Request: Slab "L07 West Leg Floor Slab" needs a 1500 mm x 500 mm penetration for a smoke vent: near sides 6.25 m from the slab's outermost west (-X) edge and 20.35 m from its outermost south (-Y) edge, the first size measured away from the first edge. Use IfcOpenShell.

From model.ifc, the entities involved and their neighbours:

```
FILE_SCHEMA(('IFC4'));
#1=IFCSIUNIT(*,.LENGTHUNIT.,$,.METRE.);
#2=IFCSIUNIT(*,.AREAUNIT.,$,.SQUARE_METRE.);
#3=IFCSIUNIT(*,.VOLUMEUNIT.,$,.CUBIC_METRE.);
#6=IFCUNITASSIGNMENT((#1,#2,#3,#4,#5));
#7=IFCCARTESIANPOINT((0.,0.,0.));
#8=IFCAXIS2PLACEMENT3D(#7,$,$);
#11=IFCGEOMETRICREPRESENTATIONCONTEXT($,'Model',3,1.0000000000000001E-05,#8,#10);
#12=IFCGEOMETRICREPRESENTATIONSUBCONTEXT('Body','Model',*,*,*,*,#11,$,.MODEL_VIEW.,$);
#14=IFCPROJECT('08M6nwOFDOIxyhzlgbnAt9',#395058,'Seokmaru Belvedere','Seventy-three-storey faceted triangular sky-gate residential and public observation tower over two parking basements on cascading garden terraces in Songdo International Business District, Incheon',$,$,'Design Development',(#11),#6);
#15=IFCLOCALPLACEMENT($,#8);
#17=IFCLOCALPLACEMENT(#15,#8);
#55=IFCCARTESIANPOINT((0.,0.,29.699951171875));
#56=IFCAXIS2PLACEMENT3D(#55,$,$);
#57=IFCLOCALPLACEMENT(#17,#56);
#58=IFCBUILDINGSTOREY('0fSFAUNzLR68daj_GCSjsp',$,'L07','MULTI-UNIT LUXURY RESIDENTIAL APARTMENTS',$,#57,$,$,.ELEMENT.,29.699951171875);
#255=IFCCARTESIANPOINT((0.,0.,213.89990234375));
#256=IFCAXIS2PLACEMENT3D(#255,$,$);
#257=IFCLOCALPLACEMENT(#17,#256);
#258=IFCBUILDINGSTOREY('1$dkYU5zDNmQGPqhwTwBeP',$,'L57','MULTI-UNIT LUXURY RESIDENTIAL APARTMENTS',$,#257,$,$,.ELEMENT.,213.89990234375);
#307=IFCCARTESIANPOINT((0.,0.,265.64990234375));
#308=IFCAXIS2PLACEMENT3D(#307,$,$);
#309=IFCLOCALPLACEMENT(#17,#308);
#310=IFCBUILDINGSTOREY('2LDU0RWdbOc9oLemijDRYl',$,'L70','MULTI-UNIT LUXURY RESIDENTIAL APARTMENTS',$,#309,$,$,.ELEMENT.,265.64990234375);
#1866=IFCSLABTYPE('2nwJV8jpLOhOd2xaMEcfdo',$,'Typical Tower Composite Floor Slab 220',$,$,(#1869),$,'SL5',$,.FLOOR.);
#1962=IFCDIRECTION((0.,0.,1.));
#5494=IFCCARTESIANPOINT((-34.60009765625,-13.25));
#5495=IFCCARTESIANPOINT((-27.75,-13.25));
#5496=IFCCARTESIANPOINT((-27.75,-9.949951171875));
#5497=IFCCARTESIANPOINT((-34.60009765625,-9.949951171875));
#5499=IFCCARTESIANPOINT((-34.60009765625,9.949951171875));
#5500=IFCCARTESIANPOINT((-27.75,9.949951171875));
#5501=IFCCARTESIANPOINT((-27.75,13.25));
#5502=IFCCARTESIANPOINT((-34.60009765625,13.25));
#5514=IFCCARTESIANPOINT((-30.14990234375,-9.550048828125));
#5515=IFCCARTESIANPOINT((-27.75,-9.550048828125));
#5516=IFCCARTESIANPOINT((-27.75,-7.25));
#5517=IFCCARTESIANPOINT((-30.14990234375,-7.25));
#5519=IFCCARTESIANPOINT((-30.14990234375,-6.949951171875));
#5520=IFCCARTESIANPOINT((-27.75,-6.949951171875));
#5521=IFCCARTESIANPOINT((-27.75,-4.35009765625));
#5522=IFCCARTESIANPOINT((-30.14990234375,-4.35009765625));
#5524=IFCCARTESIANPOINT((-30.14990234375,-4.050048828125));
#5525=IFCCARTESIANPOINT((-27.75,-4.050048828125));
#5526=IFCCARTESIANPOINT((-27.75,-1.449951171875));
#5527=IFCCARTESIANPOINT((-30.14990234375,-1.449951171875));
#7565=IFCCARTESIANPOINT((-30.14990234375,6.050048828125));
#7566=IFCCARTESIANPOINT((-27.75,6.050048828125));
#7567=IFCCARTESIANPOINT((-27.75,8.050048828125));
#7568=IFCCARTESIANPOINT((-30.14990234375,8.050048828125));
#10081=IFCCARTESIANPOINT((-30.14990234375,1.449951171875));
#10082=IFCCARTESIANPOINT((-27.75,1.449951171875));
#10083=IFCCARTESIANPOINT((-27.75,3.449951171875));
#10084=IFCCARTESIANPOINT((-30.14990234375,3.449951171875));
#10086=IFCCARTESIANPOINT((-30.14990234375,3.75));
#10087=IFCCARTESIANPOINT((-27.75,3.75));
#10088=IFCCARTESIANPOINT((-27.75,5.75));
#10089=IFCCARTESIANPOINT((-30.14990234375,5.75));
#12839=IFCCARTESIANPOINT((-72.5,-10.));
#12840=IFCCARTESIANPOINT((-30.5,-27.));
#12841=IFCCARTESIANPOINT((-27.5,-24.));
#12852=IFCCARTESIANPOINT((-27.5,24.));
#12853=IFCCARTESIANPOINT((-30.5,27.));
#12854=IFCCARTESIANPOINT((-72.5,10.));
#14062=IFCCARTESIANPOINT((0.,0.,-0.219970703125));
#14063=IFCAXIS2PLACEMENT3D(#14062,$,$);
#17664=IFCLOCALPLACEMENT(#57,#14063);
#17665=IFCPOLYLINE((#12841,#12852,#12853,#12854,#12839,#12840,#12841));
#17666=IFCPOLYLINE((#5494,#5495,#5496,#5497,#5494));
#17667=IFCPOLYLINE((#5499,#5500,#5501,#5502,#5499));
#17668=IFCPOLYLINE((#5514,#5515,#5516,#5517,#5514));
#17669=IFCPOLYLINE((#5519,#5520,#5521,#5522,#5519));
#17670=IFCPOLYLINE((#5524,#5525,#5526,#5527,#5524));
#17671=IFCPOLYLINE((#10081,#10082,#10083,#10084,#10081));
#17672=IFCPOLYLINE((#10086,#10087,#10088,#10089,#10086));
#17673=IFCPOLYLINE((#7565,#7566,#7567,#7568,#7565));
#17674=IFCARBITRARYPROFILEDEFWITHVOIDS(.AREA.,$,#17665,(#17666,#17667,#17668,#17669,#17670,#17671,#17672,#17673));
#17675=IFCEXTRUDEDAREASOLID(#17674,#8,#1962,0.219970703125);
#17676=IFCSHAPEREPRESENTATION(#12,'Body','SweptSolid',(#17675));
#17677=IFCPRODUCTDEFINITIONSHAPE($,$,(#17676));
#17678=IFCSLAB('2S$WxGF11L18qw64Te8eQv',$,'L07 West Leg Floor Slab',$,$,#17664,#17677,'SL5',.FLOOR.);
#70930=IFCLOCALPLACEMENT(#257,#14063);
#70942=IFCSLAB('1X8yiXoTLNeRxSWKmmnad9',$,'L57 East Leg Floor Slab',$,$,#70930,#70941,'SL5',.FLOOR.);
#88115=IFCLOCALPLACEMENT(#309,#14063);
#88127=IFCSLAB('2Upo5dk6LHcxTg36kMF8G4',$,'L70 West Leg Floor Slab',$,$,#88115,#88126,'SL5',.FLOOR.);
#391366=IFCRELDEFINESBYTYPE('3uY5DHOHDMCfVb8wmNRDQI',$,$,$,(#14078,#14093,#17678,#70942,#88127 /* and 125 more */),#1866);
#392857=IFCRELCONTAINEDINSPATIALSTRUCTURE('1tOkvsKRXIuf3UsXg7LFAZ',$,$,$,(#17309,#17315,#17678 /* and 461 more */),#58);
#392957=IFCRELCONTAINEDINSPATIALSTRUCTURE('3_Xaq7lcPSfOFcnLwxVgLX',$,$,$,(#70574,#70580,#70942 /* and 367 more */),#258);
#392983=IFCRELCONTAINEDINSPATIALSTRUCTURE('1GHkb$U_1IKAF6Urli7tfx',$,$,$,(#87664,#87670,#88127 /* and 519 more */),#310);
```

```python
import numpy as np
import ifcopenshell
import ifcopenshell.api.feature
import ifcopenshell.api.geometry
import ifcopenshell.api.root
import ifcopenshell.geom
import ifcopenshell.util.placement
import ifcopenshell.util.representation
import ifcopenshell.util.shape
import ifcopenshell.util.unit

model = ifcopenshell.open("model.ifc")
unit_scale = ifcopenshell.util.unit.calculate_unit_scale(model)
settings = ifcopenshell.geom.settings()


def volume(element):
    """Net volume in cubic metres, openings subtracted."""
    shape = ifcopenshell.geom.create_shape(settings, element)
    return ifcopenshell.util.shape.get_volume(shape.geometry)


slab = model.by_guid("2S$WxGF11L18qw64Te8eQv")
before = volume(slab)

# Extent in the slab's own axes, in metres. The edges named are its -X and -Y sides.
slab_shape = ifcopenshell.geom.create_shape(settings, slab)
vertices = ifcopenshell.util.shape.get_vertices(slab_shape.geometry)
x_min, y_min, bottom = vertices.min(axis=0)
top = vertices[:, 2].max()

opening = ifcopenshell.api.root.create_entity(model, ifc_class="IfcOpeningElement", name="Smoke vent opening", predefined_type="OPENING")
context = ifcopenshell.util.representation.get_context(model, "Model", "Body", "MODEL_VIEW")
width, depth = 1.5, 0.5
outline = [(0.0, 0.0), (width, 0.0), (width, depth), (0.0, depth), (0.0, 0.0)]
# Overshoot both faces by 50 mm so the cut is clean.
shape = ifcopenshell.api.geometry.add_slab_representation(
    model, context=context, depth=top - bottom + 0.1, polyline=outline
)
ifcopenshell.api.geometry.assign_representation(model, product=opening, representation=shape)

matrix = ifcopenshell.util.placement.get_local_placement(slab.ObjectPlacement)
matrix[:, 3] = matrix @ np.append(np.array([x_min + 6.25, y_min + 20.35, bottom - 0.05]) / unit_scale, 1.0)
ifcopenshell.api.geometry.edit_object_placement(model, product=opening, matrix=matrix, is_si=False)
ifcopenshell.api.feature.add_feature(model, feature=opening, element=slab)

after = volume(slab)

print(f"slab volume {before:.3f} -> {after:.3f} m3")

model.write("model_rev.ifc")
```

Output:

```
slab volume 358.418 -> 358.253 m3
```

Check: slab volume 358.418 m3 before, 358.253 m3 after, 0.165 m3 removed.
